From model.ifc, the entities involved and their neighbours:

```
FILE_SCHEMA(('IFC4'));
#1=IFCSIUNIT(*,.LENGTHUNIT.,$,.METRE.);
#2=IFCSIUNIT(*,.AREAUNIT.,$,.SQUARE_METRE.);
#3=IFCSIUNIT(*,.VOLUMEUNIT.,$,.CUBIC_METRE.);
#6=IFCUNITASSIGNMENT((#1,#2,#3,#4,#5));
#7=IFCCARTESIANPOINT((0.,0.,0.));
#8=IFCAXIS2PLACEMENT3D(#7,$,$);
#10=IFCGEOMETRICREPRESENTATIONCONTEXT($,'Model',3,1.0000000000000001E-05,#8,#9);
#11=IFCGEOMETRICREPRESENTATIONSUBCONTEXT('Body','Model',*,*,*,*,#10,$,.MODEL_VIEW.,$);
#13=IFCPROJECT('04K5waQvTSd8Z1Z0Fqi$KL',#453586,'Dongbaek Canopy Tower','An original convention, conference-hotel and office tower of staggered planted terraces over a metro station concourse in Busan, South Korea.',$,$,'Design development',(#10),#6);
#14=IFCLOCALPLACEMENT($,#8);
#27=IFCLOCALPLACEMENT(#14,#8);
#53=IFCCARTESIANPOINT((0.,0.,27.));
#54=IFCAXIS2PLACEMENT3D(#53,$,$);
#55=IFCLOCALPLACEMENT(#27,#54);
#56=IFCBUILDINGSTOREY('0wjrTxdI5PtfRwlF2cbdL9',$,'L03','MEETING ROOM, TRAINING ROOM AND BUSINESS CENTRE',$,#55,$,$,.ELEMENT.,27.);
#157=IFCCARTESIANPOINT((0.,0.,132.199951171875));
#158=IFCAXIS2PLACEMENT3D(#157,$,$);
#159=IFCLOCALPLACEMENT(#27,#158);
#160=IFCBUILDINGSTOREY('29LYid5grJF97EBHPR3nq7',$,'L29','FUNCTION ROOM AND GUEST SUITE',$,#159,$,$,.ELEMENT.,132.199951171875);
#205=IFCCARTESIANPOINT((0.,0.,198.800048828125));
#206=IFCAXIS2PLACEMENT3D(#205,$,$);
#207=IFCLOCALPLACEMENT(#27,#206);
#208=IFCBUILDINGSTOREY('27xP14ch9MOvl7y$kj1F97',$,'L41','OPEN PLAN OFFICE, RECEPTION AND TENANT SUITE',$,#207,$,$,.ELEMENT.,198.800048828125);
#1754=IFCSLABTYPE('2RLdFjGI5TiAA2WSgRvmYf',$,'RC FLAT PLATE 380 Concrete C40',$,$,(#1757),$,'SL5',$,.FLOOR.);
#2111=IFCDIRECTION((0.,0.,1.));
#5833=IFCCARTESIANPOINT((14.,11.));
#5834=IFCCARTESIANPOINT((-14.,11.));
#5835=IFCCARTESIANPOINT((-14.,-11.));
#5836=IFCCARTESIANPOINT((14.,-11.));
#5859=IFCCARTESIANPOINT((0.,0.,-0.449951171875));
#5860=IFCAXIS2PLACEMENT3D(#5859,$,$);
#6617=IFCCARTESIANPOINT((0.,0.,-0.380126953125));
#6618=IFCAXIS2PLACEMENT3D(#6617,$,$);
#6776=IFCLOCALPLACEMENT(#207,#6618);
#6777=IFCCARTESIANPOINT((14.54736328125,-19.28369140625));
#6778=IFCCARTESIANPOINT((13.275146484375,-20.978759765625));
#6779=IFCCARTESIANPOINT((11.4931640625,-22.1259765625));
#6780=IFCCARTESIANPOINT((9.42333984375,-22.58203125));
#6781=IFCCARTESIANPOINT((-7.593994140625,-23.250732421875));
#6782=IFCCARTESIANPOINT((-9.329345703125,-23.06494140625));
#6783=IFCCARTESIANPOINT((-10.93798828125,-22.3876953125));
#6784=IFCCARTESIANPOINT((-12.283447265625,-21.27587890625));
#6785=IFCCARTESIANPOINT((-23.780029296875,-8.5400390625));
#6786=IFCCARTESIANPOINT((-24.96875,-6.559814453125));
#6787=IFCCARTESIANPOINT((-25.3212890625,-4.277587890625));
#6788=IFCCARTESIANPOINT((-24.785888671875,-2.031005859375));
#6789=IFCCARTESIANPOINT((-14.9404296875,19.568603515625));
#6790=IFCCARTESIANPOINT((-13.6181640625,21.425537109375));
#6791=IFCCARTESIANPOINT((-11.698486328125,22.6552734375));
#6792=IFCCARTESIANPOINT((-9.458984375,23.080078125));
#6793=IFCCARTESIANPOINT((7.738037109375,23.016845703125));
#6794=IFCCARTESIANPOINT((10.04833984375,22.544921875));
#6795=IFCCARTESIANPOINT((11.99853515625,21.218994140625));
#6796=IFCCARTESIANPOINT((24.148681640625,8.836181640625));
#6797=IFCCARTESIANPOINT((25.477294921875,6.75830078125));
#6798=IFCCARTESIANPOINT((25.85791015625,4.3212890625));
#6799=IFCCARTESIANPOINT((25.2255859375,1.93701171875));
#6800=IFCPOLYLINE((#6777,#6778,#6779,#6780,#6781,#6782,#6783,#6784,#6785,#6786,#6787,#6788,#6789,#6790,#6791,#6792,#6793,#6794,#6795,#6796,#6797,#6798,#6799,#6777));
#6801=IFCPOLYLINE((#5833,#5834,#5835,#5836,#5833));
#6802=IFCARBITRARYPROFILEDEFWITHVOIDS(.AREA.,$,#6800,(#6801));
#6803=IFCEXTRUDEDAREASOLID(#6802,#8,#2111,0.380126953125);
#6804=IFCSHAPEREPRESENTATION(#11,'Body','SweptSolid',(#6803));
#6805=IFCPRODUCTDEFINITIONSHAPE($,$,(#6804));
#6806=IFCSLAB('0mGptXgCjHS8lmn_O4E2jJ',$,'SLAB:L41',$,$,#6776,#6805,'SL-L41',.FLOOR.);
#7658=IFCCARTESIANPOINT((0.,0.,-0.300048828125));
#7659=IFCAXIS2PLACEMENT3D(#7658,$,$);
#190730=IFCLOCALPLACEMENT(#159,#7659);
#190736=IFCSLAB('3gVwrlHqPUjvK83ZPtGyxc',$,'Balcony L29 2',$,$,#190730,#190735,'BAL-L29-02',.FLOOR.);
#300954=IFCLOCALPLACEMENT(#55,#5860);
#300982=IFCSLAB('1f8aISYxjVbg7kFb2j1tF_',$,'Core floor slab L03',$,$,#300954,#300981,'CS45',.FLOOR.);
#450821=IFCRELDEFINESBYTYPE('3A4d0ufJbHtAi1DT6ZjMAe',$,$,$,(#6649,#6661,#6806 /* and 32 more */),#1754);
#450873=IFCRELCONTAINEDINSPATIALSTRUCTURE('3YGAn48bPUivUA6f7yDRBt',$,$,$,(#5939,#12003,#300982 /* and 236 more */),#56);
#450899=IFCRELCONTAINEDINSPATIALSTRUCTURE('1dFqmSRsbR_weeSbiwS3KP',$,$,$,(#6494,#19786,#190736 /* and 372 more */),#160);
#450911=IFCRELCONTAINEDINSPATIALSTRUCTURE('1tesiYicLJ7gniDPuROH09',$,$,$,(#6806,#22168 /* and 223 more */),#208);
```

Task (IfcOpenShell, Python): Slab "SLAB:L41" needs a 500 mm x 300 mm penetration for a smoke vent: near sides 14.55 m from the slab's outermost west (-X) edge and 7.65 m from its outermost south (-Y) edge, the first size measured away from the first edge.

```python
import numpy as np
import ifcopenshell
import ifcopenshell.api.feature
import ifcopenshell.api.geometry
import ifcopenshell.api.root
import ifcopenshell.geom
import ifcopenshell.util.placement
import ifcopenshell.util.representation
import ifcopenshell.util.shape
import ifcopenshell.util.unit

model = ifcopenshell.open("model.ifc")
unit_scale = ifcopenshell.util.unit.calculate_unit_scale(model)
settings = ifcopenshell.geom.settings()


def volume(element):
    """Net volume in cubic metres, openings subtracted."""
    shape = ifcopenshell.geom.create_shape(settings, element)
    return ifcopenshell.util.shape.get_volume(shape.geometry)


slab = model.by_guid("0mGptXgCjHS8lmn_O4E2jJ")
before = volume(slab)

# Extent in the slab's own axes, in metres. The edges named are its -X and -Y sides.
slab_shape = ifcopenshell.geom.create_shape(settings, slab)
vertices = ifcopenshell.util.shape.get_vertices(slab_shape.geometry)
x_min, y_min, bottom = vertices.min(axis=0)
top = vertices[:, 2].max()

opening = ifcopenshell.api.root.create_entity(model, ifc_class="IfcOpeningElement", name="Smoke vent opening", predefined_type="OPENING")
context = ifcopenshell.util.representation.get_context(model, "Model", "Body", "MODEL_VIEW")
width, depth = 0.5, 0.3
outline = [(0.0, 0.0), (width, 0.0), (width, depth), (0.0, depth), (0.0, 0.0)]
# Overshoot both faces by 50 mm so the cut is clean.
shape = ifcopenshell.api.geometry.add_slab_representation(
    model, context=context, depth=top - bottom + 0.1, polyline=outline
)
ifcopenshell.api.geometry.assign_representation(model, product=opening, representation=shape)

matrix = ifcopenshell.util.placement.get_local_placement(slab.ObjectPlacement)
matrix[:, 3] = matrix @ np.append(np.array([x_min + 14.55, y_min + 7.65, bottom - 0.05]) / unit_scale, 1.0)
ifcopenshell.api.geometry.edit_object_placement(model, product=opening, matrix=matrix, is_si=False)
ifcopenshell.api.feature.add_feature(model, feature=opening, element=slab)

after = volume(slab)

print(f"slab volume {before:.3f} -> {after:.3f} m3")

model.write("model_updated.ifc")
```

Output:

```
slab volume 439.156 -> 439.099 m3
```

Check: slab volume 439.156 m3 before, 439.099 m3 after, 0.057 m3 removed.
